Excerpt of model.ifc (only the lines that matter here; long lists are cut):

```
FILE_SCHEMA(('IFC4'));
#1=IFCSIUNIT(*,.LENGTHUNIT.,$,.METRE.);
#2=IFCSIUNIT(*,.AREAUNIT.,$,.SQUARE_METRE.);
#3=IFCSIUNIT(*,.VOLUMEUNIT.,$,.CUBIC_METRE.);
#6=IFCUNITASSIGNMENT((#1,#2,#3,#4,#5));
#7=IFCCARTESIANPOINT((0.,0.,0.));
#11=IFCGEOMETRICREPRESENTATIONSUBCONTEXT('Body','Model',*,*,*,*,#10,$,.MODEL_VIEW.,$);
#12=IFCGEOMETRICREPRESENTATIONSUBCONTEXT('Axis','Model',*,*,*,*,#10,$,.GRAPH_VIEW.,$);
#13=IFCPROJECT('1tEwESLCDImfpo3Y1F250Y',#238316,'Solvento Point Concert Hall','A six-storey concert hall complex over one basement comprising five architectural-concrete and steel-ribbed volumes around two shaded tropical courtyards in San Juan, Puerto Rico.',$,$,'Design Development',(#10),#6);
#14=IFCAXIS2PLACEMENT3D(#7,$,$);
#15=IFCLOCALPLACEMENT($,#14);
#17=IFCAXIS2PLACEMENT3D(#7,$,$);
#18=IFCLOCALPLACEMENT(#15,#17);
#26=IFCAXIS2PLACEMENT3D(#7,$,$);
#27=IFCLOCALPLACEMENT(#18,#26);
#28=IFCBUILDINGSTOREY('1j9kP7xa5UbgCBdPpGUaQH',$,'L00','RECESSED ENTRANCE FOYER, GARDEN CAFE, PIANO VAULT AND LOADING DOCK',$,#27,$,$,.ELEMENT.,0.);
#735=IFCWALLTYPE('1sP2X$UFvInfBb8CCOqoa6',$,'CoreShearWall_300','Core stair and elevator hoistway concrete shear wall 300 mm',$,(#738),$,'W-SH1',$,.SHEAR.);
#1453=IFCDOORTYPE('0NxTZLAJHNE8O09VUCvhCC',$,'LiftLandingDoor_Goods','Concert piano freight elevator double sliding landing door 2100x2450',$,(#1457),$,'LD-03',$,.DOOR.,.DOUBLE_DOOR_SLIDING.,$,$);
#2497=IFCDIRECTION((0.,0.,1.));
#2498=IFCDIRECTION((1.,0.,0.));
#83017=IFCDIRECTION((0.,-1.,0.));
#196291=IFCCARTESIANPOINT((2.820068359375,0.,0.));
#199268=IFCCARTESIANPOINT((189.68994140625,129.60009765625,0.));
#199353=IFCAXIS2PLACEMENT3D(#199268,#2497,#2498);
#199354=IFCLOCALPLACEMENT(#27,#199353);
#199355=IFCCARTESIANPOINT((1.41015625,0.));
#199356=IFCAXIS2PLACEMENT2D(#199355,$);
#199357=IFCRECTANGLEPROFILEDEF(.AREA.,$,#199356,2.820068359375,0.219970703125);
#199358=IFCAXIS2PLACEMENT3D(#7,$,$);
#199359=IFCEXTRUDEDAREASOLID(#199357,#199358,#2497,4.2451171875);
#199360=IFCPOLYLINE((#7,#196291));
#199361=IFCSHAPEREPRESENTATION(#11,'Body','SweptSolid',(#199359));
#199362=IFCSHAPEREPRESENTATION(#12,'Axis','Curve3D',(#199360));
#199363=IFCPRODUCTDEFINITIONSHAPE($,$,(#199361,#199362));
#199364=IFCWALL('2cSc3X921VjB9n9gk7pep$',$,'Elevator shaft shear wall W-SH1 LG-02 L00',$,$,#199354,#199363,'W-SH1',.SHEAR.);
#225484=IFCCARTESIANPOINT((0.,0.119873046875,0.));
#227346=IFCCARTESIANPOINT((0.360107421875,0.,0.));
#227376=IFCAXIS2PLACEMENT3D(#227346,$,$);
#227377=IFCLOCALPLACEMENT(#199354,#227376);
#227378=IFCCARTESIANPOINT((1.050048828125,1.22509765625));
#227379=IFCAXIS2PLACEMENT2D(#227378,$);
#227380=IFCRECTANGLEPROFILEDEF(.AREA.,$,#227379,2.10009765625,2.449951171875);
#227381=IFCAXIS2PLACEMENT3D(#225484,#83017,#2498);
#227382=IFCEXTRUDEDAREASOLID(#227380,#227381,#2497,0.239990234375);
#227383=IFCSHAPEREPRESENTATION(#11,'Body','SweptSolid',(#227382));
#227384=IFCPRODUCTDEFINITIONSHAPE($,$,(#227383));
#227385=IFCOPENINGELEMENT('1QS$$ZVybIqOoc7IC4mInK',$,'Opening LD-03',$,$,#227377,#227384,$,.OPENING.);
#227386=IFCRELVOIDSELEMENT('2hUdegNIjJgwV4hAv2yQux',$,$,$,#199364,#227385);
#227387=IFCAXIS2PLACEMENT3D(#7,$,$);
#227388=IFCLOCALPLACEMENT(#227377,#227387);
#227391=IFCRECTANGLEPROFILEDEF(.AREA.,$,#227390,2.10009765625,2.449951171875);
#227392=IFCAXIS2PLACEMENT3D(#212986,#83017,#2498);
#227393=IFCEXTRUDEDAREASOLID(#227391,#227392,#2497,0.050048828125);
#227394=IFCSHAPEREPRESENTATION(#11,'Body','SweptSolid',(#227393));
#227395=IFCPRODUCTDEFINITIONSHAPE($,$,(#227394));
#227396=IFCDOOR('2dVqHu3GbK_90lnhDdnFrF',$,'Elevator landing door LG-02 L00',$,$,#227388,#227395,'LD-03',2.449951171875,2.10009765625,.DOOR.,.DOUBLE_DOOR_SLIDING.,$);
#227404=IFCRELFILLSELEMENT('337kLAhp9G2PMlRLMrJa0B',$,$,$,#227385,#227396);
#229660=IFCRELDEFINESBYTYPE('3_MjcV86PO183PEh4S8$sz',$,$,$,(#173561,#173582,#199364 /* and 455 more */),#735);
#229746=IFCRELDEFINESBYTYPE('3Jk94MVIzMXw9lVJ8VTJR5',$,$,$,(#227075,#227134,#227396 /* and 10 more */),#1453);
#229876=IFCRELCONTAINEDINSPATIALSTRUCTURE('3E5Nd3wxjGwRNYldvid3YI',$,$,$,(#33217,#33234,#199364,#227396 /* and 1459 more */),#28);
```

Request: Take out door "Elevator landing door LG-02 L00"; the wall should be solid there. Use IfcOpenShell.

```python
import ifcopenshell
import ifcopenshell.api.feature
import ifcopenshell.api.root
import ifcopenshell.geom
import ifcopenshell.util.shape

model = ifcopenshell.open("model.ifc")
settings = ifcopenshell.geom.settings()


def volume(element):
    """Net volume in cubic metres, openings subtracted."""
    shape = ifcopenshell.geom.create_shape(settings, element)
    return ifcopenshell.util.shape.get_volume(shape.geometry)


door = model.by_id(227396)
opening = door.FillsVoids[0].RelatingOpeningElement
wall = opening.VoidsElements[0].RelatingBuildingElement
before = volume(wall)

ifcopenshell.api.root.remove_product(model, product=door)
ifcopenshell.api.feature.remove_feature(model, feature=opening)

after = volume(wall)

print(f"wall volume {before:.3f} -> {after:.3f} m3")

model.write("model_rev.ifc")
```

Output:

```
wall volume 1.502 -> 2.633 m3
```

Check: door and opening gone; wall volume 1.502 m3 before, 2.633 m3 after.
